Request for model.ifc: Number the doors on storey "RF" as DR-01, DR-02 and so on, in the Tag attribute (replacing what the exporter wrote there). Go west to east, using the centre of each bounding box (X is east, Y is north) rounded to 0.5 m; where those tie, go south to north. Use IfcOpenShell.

First a look at what the model holds.

```python
import ifcopenshell
import ifcopenshell.util.element
import ifcopenshell.util.placement

model = ifcopenshell.open("model.ifc")
print(model.schema)
storey = next(s for s in model.by_type("IfcBuildingStorey") if s.Name == "RF")
doors = [e for e in ifcopenshell.util.element.get_decomposition(storey) if e.is_a("IfcDoor")]
for e in sorted(doors, key=lambda e: e.id()):
    origin = ifcopenshell.util.placement.get_local_placement(e.ObjectPlacement)[:3, 3]
    print(e.id(), e.Tag, e.Name, origin.round(2) + 0.0, sep=" | ")
```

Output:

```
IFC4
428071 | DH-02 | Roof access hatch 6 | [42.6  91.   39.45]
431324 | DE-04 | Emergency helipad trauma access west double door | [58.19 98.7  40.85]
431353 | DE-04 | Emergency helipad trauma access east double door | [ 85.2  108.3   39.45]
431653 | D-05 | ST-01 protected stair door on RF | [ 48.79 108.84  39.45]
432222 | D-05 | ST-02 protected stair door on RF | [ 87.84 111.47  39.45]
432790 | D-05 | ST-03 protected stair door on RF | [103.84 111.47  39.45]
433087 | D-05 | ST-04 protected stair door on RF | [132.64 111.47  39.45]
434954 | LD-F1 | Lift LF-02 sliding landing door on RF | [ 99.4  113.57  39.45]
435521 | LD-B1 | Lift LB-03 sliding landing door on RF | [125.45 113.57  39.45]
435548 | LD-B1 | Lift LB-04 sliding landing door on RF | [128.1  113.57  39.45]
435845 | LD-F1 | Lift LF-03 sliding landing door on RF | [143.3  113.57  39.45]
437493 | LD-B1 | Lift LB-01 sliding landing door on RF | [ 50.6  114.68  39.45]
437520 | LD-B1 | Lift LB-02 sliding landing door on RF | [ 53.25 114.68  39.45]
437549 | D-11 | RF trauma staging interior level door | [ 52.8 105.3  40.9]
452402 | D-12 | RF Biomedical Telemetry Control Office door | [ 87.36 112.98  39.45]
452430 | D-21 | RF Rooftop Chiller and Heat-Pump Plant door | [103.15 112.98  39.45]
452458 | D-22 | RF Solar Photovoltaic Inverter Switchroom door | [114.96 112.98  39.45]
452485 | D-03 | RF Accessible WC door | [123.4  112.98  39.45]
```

```python
import ifcopenshell
import ifcopenshell.geom
import ifcopenshell.util.element
import ifcopenshell.util.shape

model = ifcopenshell.open("model.ifc")
settings = ifcopenshell.geom.settings()
settings.set("use-world-coords", True)


def centre(element):
    shape = ifcopenshell.geom.create_shape(settings, element)
    return ifcopenshell.util.shape.get_bbox_centroid(shape.geometry)


storey = next(s for s in model.by_type("IfcBuildingStorey") if s.Name == "RF")
doors = [e for e in ifcopenshell.util.element.get_decomposition(storey) if e.is_a("IfcDoor")]

# Insertion points can sit at a corner or the storey origin, so sort by the geometry (in metres).
centres = {e: centre(e) for e in doors}
doors.sort(key=lambda e: (round(centres[e][0] / 0.5), centres[e][1]))

for i, e in enumerate(doors, start=1):
    number = f"DR-{i:02d}"
    e.Tag = number
    print(e.id(), number)

model.write("model-out.ifc")
```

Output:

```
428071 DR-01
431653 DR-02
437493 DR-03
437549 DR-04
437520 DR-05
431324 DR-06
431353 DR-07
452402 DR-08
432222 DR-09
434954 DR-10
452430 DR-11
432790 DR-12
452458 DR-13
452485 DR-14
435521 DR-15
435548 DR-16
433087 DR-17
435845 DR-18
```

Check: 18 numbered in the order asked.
